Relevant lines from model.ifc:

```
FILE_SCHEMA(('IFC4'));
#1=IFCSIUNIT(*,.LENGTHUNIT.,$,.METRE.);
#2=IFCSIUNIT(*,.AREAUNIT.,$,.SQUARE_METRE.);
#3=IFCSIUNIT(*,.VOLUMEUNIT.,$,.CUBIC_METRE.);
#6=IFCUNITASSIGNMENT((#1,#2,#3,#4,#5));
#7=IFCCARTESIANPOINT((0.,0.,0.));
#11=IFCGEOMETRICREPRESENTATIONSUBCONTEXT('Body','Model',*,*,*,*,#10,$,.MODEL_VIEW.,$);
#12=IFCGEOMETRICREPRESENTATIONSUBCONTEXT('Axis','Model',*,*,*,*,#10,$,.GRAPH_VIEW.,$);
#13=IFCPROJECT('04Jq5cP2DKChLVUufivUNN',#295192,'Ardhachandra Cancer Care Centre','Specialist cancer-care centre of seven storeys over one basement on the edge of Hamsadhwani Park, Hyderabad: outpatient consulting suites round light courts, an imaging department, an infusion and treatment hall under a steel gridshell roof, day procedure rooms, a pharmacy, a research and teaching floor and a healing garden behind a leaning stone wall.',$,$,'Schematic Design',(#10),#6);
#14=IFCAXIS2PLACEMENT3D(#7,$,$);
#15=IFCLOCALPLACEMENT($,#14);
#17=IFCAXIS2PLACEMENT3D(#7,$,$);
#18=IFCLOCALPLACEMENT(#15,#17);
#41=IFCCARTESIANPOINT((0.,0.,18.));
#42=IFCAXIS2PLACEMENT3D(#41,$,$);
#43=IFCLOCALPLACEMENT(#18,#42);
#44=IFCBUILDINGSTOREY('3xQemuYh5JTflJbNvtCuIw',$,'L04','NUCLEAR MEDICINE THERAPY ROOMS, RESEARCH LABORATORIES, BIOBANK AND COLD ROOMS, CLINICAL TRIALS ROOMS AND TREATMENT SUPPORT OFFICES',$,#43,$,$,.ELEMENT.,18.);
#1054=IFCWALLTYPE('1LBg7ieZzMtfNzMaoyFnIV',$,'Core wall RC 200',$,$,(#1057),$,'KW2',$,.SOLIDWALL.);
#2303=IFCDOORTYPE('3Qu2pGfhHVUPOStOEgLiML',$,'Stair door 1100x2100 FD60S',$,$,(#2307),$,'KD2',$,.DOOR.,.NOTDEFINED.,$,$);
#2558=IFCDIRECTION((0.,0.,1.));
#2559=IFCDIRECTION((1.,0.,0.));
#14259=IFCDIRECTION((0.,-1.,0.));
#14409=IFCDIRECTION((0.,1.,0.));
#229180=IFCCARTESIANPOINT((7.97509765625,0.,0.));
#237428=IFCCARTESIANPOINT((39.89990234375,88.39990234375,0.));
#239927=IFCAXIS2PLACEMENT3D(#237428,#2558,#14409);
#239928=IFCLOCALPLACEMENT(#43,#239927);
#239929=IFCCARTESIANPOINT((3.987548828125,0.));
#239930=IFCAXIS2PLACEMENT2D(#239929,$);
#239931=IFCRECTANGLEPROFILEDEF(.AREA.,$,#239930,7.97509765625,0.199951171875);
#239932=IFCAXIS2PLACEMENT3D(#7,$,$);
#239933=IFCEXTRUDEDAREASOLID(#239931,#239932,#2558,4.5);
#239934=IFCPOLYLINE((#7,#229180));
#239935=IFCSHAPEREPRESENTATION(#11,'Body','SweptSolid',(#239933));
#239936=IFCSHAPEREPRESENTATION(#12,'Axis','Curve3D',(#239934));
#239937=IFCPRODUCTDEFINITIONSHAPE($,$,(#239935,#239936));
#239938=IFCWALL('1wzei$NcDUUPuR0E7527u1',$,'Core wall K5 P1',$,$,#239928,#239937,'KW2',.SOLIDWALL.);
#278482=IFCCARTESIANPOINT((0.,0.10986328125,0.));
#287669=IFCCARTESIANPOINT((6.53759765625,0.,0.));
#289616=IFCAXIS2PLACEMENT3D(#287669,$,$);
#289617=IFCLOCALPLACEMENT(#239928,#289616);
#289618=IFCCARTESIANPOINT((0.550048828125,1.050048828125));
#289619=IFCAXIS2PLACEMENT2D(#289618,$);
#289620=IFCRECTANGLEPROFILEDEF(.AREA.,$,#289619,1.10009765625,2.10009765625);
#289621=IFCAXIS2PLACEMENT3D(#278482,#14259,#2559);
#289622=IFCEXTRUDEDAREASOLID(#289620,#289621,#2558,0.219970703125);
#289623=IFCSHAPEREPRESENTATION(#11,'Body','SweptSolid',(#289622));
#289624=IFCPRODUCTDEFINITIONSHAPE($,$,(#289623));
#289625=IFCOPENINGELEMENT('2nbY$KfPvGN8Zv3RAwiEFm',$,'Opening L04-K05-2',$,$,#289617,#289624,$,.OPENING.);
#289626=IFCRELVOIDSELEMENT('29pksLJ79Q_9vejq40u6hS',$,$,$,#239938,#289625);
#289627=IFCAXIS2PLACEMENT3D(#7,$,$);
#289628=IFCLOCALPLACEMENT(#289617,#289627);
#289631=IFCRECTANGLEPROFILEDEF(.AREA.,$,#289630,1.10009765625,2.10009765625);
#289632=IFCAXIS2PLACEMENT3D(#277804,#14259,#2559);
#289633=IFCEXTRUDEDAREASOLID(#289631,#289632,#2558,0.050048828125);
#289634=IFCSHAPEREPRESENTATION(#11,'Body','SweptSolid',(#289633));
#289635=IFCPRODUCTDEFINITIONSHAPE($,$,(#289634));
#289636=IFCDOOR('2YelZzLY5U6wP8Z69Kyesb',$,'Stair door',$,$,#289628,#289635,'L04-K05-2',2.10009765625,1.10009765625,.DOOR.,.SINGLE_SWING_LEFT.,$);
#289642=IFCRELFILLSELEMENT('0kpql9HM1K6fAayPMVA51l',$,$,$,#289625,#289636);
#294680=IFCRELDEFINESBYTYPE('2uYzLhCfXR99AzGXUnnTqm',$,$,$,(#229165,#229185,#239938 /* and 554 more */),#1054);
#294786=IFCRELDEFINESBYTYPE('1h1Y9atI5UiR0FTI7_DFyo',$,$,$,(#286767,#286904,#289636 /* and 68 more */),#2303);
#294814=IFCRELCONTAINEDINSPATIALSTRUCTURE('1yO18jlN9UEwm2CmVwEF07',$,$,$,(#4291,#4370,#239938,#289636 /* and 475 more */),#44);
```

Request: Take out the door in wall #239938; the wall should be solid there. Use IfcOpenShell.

```python
import ifcopenshell
import ifcopenshell.api.feature
import ifcopenshell.api.root
import ifcopenshell.geom
import ifcopenshell.util.shape

model = ifcopenshell.open("model.ifc")
settings = ifcopenshell.geom.settings()


def volume(element):
    """Net volume in cubic metres, openings subtracted."""
    shape = ifcopenshell.geom.create_shape(settings, element)
    return ifcopenshell.util.shape.get_volume(shape.geometry)


door = model.by_id(289636)
opening = door.FillsVoids[0].RelatingOpeningElement
wall = opening.VoidsElements[0].RelatingBuildingElement
before = volume(wall)

ifcopenshell.api.root.remove_product(model, product=door)
ifcopenshell.api.feature.remove_feature(model, feature=opening)

after = volume(wall)

print(f"wall volume {before:.3f} -> {after:.3f} m3")

model.write("model_v2.ifc")
```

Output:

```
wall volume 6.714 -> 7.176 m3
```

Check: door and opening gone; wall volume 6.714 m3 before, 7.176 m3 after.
